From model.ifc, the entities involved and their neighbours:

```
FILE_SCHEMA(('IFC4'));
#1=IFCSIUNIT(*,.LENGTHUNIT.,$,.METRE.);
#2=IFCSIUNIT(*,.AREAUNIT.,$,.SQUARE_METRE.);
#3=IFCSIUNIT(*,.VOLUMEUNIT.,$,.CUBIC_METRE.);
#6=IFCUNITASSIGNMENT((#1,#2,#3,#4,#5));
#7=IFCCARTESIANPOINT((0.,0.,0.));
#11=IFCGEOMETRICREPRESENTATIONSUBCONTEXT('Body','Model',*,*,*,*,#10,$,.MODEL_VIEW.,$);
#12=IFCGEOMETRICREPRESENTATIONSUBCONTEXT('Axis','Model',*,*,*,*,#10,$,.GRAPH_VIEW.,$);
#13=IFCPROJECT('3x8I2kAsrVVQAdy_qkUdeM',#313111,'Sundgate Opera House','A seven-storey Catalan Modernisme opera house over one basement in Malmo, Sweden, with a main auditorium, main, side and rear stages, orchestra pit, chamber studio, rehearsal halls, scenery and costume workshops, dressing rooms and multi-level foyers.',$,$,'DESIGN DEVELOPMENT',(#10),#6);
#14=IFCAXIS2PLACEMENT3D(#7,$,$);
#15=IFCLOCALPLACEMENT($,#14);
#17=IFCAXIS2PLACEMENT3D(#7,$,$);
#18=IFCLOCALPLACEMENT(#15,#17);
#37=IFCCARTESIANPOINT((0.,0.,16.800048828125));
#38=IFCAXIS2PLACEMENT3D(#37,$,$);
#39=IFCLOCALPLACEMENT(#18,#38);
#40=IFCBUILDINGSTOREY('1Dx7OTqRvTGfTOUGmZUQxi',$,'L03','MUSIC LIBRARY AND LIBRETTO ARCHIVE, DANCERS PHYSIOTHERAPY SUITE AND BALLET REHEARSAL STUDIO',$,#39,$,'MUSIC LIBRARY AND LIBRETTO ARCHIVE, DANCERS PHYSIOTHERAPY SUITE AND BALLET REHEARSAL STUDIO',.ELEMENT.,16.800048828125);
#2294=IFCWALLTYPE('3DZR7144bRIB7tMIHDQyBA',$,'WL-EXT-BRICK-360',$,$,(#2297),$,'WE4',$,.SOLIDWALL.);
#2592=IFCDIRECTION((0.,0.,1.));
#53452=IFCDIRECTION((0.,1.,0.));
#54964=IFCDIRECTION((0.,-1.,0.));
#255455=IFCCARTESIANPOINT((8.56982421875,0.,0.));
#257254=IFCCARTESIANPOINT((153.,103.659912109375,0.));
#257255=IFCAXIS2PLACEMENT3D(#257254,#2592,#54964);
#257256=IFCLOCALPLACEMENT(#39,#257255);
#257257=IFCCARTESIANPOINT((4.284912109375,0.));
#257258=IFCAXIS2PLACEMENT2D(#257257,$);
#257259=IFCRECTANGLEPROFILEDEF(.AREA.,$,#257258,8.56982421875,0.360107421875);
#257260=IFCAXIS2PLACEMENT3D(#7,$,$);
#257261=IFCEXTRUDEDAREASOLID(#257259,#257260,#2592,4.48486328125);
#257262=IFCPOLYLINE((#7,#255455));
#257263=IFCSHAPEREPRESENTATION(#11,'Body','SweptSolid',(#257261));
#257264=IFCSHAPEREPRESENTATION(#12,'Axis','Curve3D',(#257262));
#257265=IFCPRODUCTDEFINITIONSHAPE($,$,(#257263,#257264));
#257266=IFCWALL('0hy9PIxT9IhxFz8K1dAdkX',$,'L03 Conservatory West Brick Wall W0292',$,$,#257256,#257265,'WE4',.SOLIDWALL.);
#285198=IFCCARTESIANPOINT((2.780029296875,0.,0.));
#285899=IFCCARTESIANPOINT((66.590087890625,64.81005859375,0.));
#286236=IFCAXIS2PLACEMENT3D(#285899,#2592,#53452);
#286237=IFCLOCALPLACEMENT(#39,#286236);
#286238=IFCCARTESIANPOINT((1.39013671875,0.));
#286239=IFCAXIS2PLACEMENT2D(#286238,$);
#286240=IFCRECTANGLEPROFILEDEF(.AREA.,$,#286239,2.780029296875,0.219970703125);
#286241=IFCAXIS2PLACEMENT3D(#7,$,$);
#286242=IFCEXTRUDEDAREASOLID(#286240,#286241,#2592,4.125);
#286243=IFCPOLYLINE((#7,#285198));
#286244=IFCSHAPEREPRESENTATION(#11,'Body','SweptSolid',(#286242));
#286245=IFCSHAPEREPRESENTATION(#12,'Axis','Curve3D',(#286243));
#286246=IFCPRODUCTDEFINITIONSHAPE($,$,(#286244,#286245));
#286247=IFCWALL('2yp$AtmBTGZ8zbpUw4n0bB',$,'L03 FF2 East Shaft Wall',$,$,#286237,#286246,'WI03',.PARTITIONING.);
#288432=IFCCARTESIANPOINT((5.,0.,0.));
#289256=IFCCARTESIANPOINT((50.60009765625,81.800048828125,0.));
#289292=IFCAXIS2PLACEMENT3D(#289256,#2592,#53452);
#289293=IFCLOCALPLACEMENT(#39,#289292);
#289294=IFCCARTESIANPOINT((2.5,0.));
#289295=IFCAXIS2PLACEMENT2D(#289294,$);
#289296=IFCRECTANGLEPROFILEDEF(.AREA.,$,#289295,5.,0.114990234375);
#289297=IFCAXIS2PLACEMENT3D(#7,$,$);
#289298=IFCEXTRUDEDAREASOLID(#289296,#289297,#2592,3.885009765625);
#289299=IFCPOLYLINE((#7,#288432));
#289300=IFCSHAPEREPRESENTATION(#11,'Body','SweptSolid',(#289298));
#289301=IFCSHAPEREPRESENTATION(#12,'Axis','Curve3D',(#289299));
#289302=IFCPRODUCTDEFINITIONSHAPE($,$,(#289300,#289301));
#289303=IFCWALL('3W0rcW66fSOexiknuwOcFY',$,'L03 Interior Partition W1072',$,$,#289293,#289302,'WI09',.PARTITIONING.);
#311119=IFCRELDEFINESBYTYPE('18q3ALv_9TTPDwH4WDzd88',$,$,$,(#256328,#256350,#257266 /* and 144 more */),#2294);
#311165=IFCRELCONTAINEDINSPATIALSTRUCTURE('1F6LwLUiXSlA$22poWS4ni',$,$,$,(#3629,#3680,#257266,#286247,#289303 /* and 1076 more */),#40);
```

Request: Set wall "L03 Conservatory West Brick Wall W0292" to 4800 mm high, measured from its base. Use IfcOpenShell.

```python
import ifcopenshell
import ifcopenshell.geom
import ifcopenshell.util.representation
import ifcopenshell.util.shape

model = ifcopenshell.open("model.ifc")
settings = ifcopenshell.geom.settings()


def volume(element):
    """Net volume in cubic metres, openings subtracted."""
    shape = ifcopenshell.geom.create_shape(settings, element)
    return ifcopenshell.util.shape.get_volume(shape.geometry)


wall = model.by_guid("0hy9PIxT9IhxFz8K1dAdkX")
before = volume(wall)

body = ifcopenshell.util.representation.get_representation(wall, "Model", "Body")
solid = body.Items[0]
old_height = solid.Depth
solid.Depth = 4.8
after = volume(wall)

print(f"height {old_height:g} -> {solid.Depth:g}, volume {before:.3f} -> {after:.3f} m3")

model.write("model_updated.ifc")
```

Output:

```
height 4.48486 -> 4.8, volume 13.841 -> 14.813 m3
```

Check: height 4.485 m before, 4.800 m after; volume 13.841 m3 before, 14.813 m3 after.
